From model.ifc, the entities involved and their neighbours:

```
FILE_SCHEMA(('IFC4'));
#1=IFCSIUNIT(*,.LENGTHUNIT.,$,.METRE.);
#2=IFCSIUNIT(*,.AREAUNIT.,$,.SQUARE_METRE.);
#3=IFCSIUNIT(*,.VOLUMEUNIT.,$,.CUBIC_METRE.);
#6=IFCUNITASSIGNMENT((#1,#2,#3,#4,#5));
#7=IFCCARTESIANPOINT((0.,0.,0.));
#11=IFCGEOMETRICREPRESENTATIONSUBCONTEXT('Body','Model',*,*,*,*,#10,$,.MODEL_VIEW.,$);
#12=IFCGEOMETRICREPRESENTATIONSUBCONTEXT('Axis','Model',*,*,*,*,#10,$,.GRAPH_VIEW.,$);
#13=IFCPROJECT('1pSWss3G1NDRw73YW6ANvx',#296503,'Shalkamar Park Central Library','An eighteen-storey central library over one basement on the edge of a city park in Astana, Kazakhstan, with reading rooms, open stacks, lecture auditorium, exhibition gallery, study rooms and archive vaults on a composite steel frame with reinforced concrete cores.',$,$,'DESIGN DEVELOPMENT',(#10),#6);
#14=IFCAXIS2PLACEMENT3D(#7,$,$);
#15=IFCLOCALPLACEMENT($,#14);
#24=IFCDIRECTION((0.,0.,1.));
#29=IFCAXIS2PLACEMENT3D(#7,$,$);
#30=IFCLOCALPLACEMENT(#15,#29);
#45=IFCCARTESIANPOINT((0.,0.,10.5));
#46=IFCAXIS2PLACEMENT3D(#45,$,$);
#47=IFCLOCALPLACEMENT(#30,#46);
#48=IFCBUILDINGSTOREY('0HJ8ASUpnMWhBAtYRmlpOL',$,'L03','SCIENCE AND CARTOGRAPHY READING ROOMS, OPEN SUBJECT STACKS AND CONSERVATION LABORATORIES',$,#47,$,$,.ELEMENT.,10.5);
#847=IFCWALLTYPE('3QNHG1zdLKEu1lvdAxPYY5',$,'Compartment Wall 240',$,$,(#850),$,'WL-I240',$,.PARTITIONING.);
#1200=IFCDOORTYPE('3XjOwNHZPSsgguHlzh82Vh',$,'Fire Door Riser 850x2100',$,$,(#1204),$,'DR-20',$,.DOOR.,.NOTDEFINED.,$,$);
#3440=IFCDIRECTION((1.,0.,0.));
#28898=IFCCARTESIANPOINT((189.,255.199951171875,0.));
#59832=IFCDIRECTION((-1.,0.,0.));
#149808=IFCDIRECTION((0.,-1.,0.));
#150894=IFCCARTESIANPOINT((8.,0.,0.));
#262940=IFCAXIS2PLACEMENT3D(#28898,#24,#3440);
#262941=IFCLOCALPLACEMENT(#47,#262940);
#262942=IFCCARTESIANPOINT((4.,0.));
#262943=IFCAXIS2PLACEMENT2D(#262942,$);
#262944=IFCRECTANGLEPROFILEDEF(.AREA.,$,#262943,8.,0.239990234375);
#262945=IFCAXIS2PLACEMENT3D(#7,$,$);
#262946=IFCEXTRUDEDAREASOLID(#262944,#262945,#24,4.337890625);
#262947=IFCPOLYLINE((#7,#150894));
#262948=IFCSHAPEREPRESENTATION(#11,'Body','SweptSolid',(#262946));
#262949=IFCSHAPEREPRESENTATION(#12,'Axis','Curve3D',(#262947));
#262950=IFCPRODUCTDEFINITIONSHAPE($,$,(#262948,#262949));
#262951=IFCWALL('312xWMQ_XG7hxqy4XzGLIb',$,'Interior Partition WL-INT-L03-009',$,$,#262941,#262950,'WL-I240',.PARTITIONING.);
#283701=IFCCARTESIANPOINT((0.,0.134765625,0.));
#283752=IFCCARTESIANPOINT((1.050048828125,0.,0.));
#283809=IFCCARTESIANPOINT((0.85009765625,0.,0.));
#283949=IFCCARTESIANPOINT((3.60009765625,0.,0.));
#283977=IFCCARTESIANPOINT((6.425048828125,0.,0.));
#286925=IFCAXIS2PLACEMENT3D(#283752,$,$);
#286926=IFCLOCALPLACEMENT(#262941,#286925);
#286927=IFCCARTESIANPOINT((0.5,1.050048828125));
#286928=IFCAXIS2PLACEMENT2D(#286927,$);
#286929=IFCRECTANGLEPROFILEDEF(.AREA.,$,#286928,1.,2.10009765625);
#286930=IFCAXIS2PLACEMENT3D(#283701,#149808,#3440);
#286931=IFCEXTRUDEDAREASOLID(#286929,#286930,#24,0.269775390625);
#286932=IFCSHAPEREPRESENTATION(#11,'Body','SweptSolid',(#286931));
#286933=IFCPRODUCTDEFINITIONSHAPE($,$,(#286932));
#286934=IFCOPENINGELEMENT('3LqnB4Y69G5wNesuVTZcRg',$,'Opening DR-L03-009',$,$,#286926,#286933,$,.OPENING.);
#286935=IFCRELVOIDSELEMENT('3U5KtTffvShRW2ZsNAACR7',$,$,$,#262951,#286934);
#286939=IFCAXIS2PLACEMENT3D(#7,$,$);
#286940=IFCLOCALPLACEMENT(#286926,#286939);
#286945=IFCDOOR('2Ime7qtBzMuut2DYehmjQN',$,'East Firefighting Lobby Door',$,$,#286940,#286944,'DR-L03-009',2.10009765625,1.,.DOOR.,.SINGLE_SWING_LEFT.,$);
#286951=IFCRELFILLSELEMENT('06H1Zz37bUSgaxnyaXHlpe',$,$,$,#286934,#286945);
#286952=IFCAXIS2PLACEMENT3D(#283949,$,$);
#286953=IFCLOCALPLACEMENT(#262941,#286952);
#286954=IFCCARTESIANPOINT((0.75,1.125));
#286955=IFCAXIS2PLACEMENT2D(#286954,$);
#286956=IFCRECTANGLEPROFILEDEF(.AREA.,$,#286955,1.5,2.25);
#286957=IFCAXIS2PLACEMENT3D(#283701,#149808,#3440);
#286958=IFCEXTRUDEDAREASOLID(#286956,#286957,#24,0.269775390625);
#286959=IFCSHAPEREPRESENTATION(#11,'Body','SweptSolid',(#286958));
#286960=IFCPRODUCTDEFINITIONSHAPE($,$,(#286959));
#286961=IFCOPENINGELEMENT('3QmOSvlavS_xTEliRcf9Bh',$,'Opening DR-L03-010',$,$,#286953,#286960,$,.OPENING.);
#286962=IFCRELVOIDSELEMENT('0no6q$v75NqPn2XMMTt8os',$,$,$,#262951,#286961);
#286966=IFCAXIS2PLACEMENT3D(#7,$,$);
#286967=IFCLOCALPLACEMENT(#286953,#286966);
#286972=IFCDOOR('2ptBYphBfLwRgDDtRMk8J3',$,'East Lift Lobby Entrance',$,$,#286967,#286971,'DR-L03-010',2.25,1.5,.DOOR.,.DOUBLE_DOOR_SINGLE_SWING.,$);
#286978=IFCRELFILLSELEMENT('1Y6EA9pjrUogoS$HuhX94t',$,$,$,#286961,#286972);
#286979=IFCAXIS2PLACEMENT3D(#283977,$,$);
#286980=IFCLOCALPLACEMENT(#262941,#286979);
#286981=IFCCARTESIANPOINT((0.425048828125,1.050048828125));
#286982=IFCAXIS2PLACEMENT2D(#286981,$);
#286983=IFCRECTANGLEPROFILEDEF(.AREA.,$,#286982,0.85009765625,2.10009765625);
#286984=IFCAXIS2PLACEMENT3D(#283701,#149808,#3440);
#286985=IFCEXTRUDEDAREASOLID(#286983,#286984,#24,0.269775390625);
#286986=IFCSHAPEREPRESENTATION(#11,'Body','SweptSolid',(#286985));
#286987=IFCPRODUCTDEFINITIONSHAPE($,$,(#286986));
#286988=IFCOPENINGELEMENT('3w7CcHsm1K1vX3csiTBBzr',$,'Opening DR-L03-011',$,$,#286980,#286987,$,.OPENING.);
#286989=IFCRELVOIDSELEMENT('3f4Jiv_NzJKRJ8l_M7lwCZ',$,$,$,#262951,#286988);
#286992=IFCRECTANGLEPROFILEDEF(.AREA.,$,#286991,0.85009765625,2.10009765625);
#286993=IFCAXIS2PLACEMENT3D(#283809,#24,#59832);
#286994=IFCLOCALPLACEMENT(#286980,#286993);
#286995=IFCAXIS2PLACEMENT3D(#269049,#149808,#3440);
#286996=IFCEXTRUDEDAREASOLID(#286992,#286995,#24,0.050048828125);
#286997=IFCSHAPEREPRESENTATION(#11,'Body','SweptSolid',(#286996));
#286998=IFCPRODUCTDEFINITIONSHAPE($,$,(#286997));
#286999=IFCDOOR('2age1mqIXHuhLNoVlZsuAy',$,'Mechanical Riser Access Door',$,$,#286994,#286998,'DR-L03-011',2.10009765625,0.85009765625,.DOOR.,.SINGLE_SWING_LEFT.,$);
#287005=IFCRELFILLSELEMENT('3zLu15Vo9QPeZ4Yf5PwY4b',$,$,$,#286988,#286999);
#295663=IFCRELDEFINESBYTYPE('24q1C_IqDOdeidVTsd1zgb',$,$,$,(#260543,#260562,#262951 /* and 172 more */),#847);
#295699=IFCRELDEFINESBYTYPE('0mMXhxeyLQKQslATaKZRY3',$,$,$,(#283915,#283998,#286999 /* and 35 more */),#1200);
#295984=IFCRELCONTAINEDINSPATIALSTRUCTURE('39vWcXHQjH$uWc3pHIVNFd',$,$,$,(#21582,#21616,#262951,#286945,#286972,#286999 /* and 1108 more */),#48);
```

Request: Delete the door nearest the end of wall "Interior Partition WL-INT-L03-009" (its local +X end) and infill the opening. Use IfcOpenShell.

```python
import ifcopenshell
import ifcopenshell.api.feature
import ifcopenshell.api.root
import ifcopenshell.geom
import ifcopenshell.util.shape

model = ifcopenshell.open("model.ifc")
settings = ifcopenshell.geom.settings()


def volume(element):
    """Net volume in cubic metres, openings subtracted."""
    shape = ifcopenshell.geom.create_shape(settings, element)
    return ifcopenshell.util.shape.get_volume(shape.geometry)


door = model.by_guid("2age1mqIXHuhLNoVlZsuAy")
opening = door.FillsVoids[0].RelatingOpeningElement
wall = opening.VoidsElements[0].RelatingBuildingElement
before = volume(wall)

ifcopenshell.api.root.remove_product(model, product=door)
ifcopenshell.api.feature.remove_feature(model, feature=opening)

after = volume(wall)

print(f"wall volume {before:.3f} -> {after:.3f} m3")

model.write("model-out.ifc")
```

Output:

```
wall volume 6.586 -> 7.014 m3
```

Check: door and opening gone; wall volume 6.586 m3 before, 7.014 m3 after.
